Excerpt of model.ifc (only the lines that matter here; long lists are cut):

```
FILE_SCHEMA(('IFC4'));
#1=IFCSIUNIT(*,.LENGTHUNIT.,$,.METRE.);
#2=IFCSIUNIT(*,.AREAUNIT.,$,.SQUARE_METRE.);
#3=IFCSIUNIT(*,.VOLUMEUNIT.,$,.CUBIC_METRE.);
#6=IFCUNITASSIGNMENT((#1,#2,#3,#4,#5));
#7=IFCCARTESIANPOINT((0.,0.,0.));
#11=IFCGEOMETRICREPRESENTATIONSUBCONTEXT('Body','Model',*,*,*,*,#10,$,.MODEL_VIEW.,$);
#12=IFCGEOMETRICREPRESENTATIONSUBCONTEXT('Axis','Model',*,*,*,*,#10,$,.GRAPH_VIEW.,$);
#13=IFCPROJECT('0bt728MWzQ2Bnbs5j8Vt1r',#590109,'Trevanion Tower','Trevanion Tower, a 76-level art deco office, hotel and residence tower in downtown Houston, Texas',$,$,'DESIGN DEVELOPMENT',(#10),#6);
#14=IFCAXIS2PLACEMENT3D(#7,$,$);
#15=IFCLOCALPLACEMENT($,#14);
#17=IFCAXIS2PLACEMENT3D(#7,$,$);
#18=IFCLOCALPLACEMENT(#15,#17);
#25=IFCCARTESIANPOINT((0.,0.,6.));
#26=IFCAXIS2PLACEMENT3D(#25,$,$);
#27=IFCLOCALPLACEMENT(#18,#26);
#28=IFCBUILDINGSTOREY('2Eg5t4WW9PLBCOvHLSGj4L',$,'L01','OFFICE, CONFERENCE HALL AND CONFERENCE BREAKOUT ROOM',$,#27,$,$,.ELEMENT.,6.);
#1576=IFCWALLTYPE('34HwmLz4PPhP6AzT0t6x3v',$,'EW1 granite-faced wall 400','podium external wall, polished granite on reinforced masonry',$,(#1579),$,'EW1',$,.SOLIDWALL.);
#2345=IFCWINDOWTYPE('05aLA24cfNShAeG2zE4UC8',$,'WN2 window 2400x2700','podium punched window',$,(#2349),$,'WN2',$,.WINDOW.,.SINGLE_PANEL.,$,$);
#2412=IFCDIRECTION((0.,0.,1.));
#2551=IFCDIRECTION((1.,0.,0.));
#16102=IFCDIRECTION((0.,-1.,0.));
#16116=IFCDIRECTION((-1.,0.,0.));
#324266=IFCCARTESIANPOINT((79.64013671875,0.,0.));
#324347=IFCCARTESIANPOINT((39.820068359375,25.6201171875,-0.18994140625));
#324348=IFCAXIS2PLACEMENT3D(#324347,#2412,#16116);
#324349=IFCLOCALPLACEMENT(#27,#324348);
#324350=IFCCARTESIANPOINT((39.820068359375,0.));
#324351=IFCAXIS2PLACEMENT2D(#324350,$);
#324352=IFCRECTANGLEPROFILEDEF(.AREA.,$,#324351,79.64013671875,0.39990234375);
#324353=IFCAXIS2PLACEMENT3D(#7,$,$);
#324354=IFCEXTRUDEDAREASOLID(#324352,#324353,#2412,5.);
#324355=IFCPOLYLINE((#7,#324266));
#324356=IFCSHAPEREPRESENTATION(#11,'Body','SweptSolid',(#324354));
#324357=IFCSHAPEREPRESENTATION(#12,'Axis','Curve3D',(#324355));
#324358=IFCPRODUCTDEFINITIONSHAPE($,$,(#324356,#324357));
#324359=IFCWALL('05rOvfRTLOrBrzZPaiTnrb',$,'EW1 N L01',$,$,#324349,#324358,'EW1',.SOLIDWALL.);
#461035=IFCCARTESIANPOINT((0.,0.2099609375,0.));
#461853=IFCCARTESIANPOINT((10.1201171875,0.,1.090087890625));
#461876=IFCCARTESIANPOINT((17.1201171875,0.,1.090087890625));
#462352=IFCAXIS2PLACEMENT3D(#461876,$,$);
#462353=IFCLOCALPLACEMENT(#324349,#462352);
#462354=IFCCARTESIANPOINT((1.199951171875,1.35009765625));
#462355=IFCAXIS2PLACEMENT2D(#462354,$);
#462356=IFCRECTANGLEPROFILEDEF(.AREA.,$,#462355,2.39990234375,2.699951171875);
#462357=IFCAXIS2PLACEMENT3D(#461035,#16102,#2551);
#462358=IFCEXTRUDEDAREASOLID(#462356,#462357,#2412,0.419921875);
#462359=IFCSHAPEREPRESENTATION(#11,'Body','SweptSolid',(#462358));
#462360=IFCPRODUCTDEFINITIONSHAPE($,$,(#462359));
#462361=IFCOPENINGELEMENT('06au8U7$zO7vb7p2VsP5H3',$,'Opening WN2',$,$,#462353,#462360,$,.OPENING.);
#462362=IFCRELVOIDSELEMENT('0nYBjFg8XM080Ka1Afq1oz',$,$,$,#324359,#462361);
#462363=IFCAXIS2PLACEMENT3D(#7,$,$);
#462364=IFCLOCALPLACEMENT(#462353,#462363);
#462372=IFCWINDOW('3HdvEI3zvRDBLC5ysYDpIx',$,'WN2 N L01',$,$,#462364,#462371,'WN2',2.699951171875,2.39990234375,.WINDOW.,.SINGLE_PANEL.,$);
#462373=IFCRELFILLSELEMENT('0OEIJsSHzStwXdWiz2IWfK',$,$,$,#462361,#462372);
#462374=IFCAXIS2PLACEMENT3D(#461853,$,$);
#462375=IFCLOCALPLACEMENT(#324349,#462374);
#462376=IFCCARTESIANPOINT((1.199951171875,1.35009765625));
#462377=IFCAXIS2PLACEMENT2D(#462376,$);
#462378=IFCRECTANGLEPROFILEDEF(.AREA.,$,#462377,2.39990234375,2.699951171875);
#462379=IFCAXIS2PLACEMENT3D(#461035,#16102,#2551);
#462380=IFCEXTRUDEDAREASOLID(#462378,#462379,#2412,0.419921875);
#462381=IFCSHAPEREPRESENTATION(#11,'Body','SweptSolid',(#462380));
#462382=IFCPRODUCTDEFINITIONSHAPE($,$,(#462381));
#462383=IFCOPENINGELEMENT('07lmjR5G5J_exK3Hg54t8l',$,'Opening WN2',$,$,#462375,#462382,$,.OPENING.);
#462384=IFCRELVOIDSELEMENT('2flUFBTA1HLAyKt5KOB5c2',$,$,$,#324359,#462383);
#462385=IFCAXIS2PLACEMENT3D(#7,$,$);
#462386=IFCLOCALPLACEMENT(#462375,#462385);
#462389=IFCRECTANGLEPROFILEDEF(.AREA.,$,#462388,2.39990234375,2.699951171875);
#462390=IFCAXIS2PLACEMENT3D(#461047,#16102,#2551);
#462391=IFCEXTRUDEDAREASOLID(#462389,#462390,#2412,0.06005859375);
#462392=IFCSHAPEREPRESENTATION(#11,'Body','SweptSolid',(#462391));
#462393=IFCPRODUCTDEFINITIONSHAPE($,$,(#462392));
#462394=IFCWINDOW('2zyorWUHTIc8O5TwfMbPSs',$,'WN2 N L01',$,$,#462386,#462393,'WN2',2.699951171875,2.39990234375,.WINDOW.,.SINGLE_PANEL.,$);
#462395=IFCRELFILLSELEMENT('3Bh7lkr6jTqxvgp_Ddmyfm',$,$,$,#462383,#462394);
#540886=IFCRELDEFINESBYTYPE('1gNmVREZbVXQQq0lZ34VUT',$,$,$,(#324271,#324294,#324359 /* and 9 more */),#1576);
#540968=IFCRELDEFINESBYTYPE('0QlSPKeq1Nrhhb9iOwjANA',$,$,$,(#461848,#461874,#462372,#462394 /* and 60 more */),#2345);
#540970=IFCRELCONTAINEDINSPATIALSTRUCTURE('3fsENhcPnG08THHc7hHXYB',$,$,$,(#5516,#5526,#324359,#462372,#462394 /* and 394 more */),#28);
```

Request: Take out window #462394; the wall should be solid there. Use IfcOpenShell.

```python
import ifcopenshell
import ifcopenshell.api.feature
import ifcopenshell.api.root
import ifcopenshell.geom
import ifcopenshell.util.shape

model = ifcopenshell.open("model.ifc")
settings = ifcopenshell.geom.settings()


def volume(element):
    """Net volume in cubic metres, openings subtracted."""
    shape = ifcopenshell.geom.create_shape(settings, element)
    return ifcopenshell.util.shape.get_volume(shape.geometry)


window = model.by_id(462394)
opening = window.FillsVoids[0].RelatingOpeningElement
wall = opening.VoidsElements[0].RelatingBuildingElement
before = volume(wall)

ifcopenshell.api.root.remove_product(model, product=window)
ifcopenshell.api.feature.remove_feature(model, feature=opening)

after = volume(wall)

print(f"wall volume {before:.3f} -> {after:.3f} m3")

model.write("model-out.ifc")
```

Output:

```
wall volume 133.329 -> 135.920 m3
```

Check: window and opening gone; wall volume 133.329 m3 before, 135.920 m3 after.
